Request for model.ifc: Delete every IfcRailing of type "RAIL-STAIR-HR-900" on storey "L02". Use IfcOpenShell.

First a look at what the model holds.

```python
import ifcopenshell
import ifcopenshell.util.element

model = ifcopenshell.open("model.ifc")
print(model.schema)
storey = next(s for s in model.by_type("IfcBuildingStorey") if s.Name == "L02")
railings = [e for e in ifcopenshell.util.element.get_decomposition(storey) if e.is_a("IfcRailing")]
seen = {}
for e in railings:
    element_type = ifcopenshell.util.element.get_type(e)
    name = element_type.Name if element_type not in (None, e) else None
    seen[name] = seen.get(name, 0) + 1
for name, count in sorted(seen.items(), key=str):
    print(count, "x", name)
```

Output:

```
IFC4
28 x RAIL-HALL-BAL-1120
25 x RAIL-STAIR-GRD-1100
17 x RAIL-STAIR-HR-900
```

```python
import ifcopenshell
import ifcopenshell.api.root
import ifcopenshell.util.element

model = ifcopenshell.open("model.ifc")

storey = next(s for s in model.by_type("IfcBuildingStorey") if s.Name == "L02")
railings = [e for e in ifcopenshell.util.element.get_decomposition(storey) if e.is_a("IfcRailing")]
targets = [e for e in railings if (t := ifcopenshell.util.element.get_type(e)) not in (None, e) and t.Name == "RAIL-STAIR-HR-900"]

for e in targets:
    ifcopenshell.api.root.remove_product(model, product=e)
print(len(targets), "removed")

model.write("model_edited.ifc")
```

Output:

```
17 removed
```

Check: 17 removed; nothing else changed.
